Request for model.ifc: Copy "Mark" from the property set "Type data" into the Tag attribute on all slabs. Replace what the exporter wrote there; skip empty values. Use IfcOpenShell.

First a look at what the model holds.

```python
import ifcopenshell
import ifcopenshell.util.element

model = ifcopenshell.open("model.ifc")
print(model.schema)
slabs = model.by_type("IfcSlab")
print(len(slabs), "slabs")
for e in slabs[:8]:
    source = ifcopenshell.util.element.get_pset(e, "Type data", "Mark")
    target = e.Tag
    print(e.id(), repr(source), repr(target), sep=" | ")
```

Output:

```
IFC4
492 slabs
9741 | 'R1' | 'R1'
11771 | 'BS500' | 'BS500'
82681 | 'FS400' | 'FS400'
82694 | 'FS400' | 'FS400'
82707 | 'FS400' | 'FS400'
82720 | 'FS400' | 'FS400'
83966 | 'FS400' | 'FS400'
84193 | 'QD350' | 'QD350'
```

```python
import ifcopenshell
import ifcopenshell.util.element

model = ifcopenshell.open("model.ifc")

count = 0
for e in model.by_type("IfcSlab"):
    value = ifcopenshell.util.element.get_pset(e, "Type data", "Mark")
    current = e.Tag
    if not value or not value.strip() or current == value:
        continue
    e.Tag = value
    count += 1

print(count, "slabs updated")

model.write("model_edited.ifc")
```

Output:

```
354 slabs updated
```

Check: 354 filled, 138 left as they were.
